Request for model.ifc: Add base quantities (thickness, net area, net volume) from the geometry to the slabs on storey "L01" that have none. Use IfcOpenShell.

First a look at what the model holds.

```python
import ifcopenshell
import ifcopenshell.util.element
import ifcopenshell.util.unit

model = ifcopenshell.open("model.ifc")
print(model.schema)
for unit_type in ("LENGTHUNIT", "AREAUNIT", "VOLUMEUNIT"):
    print(unit_type, ifcopenshell.util.unit.calculate_unit_scale(model, unit_type))
storey = next(s for s in model.by_type("IfcBuildingStorey") if s.Name == "L01")
slabs = [e for e in ifcopenshell.util.element.get_decomposition(storey) if e.is_a("IfcSlab")]
for e in sorted(slabs, key=lambda e: e.id()):
    print(e.id(), e.is_a(), e.Name, list(ifcopenshell.util.element.get_psets(e, qtos_only=True)), sep=" | ")
```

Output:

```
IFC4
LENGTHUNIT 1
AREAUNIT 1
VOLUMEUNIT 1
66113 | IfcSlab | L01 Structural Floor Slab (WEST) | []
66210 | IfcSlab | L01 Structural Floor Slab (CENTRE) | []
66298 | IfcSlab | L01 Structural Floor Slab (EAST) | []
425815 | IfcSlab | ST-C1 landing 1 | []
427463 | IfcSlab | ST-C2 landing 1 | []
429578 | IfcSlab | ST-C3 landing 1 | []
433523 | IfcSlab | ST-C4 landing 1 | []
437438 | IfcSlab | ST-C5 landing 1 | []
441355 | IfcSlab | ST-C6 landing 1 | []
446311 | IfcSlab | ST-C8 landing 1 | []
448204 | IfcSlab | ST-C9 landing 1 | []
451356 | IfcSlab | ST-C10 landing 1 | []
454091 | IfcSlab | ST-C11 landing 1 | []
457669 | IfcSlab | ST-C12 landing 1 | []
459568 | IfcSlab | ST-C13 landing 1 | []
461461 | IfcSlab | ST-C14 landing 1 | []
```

```python
import ifcopenshell
import ifcopenshell.api.pset
import ifcopenshell.geom
import ifcopenshell.util.element
import ifcopenshell.util.shape
import ifcopenshell.util.unit

model = ifcopenshell.open("model.ifc")
unit_scale = ifcopenshell.util.unit.calculate_unit_scale(model)
area_scale = ifcopenshell.util.unit.calculate_unit_scale(model, "AREAUNIT")
volume_scale = ifcopenshell.util.unit.calculate_unit_scale(model, "VOLUMEUNIT")
settings = ifcopenshell.geom.settings()

storey = next(s for s in model.by_type("IfcBuildingStorey") if s.Name == "L01")
slabs = [e for e in ifcopenshell.util.element.get_decomposition(storey) if e.is_a("IfcSlab")]

for e in sorted(slabs, key=lambda e: e.id()):
    if ifcopenshell.util.element.get_psets(e, qtos_only=True, should_inherit=False):
        continue
    # Geometry comes back in metres, in the element's own axes.
    shape = ifcopenshell.geom.create_shape(settings, e)
    values = {
        "Width": ifcopenshell.util.shape.get_z(shape.geometry) / unit_scale,
        "NetArea": ifcopenshell.util.shape.get_footprint_area(shape.geometry) / area_scale,
        "NetVolume": ifcopenshell.util.shape.get_volume(shape.geometry) / volume_scale,
    }
    qto = ifcopenshell.api.pset.add_qto(model, product=e, name="Qto_SlabBaseQuantities")
    ifcopenshell.api.pset.edit_qto(model, qto=qto, properties=values)
    print(e.id(), {k: round(v, 3) for k, v in values.items()})

model.write("model_updated.ifc")
```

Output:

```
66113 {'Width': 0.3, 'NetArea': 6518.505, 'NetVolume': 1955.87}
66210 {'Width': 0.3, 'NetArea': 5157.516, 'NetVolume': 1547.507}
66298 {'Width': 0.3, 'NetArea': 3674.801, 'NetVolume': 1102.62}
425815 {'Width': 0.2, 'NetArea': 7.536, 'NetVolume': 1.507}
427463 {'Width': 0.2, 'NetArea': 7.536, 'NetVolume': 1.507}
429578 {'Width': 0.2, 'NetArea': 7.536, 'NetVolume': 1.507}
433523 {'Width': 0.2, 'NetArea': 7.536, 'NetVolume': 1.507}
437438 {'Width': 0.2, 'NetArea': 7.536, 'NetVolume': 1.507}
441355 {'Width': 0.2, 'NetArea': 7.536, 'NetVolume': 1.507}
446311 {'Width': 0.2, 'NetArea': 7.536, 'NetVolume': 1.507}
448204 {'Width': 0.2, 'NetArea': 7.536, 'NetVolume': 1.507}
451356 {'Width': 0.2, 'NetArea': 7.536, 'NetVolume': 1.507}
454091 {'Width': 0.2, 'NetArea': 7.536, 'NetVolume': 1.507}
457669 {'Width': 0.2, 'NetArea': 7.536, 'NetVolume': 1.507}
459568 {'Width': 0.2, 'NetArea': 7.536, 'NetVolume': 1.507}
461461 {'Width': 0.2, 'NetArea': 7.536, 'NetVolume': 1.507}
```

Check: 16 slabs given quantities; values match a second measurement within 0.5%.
